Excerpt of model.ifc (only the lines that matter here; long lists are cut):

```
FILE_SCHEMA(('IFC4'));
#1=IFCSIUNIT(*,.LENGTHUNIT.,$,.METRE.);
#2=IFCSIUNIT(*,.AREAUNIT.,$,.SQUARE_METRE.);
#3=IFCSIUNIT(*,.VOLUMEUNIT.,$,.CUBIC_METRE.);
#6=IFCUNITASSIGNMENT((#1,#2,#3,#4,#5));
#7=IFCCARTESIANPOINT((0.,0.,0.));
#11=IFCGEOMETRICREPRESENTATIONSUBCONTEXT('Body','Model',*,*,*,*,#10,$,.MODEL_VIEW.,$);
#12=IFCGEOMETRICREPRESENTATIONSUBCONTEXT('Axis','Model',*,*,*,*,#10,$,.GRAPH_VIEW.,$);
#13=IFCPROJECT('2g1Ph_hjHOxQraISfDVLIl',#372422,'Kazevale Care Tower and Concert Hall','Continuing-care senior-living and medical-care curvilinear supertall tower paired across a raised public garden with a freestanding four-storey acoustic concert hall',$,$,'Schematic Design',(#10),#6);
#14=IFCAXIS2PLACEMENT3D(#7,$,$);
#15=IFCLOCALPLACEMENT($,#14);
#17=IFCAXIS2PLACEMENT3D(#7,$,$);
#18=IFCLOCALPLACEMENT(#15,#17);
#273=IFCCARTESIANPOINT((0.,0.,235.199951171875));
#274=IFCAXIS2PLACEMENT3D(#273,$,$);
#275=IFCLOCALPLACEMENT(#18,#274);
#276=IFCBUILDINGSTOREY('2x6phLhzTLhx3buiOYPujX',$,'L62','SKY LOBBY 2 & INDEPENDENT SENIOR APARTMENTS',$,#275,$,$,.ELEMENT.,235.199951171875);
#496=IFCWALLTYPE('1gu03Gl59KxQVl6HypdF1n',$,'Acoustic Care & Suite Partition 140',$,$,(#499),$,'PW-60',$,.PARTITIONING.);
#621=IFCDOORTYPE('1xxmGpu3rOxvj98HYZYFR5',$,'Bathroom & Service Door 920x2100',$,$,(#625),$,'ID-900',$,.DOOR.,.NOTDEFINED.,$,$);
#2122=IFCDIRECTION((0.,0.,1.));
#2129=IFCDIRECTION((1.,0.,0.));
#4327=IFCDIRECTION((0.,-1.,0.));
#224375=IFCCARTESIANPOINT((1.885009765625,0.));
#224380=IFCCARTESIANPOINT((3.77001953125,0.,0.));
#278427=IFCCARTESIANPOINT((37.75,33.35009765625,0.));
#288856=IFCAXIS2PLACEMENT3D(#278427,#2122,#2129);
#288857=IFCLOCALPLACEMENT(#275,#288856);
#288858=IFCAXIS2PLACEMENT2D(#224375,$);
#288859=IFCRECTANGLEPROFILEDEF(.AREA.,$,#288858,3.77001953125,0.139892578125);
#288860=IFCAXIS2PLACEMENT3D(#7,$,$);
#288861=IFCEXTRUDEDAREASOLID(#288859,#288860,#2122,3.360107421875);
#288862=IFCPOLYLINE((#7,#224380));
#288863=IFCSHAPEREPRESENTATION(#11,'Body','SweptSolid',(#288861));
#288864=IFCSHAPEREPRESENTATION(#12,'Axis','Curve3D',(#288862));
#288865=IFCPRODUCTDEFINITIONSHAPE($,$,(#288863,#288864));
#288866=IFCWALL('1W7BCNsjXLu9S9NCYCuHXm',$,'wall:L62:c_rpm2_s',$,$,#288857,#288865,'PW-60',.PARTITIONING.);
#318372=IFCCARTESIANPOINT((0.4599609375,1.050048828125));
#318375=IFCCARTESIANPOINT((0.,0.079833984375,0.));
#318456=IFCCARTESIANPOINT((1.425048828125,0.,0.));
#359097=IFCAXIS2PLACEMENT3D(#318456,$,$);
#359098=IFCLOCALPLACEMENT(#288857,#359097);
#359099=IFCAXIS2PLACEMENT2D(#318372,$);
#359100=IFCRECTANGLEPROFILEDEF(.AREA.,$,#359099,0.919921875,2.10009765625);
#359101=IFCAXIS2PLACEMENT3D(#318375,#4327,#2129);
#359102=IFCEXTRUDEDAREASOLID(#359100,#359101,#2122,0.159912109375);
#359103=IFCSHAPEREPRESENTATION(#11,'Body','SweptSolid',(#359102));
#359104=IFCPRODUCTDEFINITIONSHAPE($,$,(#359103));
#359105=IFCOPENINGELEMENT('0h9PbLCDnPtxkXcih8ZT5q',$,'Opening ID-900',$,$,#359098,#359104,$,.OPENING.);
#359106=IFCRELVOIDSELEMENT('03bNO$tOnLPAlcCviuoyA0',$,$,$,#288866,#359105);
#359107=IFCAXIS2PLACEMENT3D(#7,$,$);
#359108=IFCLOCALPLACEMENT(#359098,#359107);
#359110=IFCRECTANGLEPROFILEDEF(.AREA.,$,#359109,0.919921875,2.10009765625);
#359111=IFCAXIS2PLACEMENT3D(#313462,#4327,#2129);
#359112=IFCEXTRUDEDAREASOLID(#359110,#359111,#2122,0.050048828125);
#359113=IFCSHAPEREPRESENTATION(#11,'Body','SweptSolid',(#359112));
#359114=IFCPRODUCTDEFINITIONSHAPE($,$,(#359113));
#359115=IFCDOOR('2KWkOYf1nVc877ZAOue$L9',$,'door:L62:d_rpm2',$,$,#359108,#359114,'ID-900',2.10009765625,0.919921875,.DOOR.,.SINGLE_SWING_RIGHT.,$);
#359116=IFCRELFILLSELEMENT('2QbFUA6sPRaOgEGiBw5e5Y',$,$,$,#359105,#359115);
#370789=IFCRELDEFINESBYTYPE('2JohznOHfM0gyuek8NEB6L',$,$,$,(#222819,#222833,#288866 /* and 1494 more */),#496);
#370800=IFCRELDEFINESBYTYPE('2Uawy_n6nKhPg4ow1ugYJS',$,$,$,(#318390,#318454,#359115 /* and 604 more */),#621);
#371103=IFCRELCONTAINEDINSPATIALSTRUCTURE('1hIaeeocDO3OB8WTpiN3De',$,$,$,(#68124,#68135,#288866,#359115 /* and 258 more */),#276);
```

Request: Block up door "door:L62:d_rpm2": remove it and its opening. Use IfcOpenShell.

```python
import ifcopenshell
import ifcopenshell.api.feature
import ifcopenshell.api.root
import ifcopenshell.geom
import ifcopenshell.util.shape

model = ifcopenshell.open("model.ifc")
settings = ifcopenshell.geom.settings()


def volume(element):
    """Net volume in cubic metres, openings subtracted."""
    shape = ifcopenshell.geom.create_shape(settings, element)
    return ifcopenshell.util.shape.get_volume(shape.geometry)


door = model.by_id(359115)
opening = door.FillsVoids[0].RelatingOpeningElement
wall = opening.VoidsElements[0].RelatingBuildingElement
before = volume(wall)

ifcopenshell.api.root.remove_product(model, product=door)
ifcopenshell.api.feature.remove_feature(model, feature=opening)

after = volume(wall)

print(f"wall volume {before:.3f} -> {after:.3f} m3")

model.write("model-out.ifc")
```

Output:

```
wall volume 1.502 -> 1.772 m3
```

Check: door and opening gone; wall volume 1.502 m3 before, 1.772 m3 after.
